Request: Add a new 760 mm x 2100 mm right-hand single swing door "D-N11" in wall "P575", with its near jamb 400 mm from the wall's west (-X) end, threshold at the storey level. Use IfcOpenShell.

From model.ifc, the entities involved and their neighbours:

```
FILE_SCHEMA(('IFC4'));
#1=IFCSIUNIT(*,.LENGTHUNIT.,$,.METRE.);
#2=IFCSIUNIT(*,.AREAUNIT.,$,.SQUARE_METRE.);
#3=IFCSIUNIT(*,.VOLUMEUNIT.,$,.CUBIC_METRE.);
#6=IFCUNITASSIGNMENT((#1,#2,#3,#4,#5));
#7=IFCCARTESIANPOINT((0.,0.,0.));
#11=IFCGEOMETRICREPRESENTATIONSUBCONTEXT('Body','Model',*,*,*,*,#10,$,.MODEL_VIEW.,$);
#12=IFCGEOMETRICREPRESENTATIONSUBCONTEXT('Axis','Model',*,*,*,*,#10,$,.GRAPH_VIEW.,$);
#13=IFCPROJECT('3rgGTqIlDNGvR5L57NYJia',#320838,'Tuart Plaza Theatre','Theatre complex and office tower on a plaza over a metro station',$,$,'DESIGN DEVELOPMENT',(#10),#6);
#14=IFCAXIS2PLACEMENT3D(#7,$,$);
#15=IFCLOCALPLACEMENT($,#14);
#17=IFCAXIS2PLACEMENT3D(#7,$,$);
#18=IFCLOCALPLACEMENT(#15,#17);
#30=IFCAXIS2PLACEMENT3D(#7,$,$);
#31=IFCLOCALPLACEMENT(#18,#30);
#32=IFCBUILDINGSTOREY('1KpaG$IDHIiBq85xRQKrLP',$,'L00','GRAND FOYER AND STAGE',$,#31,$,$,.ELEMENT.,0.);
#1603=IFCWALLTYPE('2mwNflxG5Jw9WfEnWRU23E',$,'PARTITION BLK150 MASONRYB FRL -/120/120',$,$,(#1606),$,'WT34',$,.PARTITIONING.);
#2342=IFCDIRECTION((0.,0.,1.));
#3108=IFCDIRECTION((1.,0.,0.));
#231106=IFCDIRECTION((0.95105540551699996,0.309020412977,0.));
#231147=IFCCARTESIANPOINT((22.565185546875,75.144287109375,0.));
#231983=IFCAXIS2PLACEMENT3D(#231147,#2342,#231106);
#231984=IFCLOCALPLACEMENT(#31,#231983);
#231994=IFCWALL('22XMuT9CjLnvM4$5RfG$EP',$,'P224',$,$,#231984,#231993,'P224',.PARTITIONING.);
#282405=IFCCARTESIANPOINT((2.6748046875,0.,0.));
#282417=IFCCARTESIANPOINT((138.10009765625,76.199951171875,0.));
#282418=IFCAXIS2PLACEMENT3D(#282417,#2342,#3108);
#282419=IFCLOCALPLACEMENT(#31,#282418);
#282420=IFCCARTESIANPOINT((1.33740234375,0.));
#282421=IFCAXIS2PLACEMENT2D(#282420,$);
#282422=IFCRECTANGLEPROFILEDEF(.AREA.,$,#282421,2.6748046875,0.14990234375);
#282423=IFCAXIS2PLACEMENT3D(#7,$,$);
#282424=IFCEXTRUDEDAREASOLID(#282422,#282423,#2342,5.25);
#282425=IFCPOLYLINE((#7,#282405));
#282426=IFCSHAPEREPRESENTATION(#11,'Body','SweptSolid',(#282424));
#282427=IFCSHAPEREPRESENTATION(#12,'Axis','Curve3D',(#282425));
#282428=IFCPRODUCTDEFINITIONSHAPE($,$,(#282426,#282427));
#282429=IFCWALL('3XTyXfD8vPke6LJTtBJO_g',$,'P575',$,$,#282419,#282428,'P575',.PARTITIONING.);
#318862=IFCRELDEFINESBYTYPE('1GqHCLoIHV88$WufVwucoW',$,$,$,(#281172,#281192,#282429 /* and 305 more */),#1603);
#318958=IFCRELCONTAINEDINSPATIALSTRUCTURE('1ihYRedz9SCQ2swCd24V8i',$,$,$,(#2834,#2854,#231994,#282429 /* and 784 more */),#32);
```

```python
import numpy as np
import ifcopenshell
import ifcopenshell.api.feature
import ifcopenshell.api.geometry
import ifcopenshell.api.root
import ifcopenshell.api.spatial
import ifcopenshell.geom
import ifcopenshell.util.element
import ifcopenshell.util.placement
import ifcopenshell.util.representation
import ifcopenshell.util.shape
import ifcopenshell.util.unit

model = ifcopenshell.open("model.ifc")
unit_scale = ifcopenshell.util.unit.calculate_unit_scale(model)
settings = ifcopenshell.geom.settings()


def volume(element):
    """Net volume in cubic metres, openings subtracted."""
    shape = ifcopenshell.geom.create_shape(settings, element)
    return ifcopenshell.util.shape.get_volume(shape.geometry)


wall = model.by_id(282429)
storey = ifcopenshell.util.element.get_container(wall, ifc_class="IfcBuildingStorey")
context = ifcopenshell.util.representation.get_context(model, "Model", "Body", "MODEL_VIEW")
before = volume(wall)

width, height, from_end, sill = 0.76, 2.1, 0.4, 0.0  # metres

# The wall runs along its own X axis, and the end named is its -X end.
wall_shape = ifcopenshell.geom.create_shape(settings, wall)
x, y, z = ifcopenshell.util.shape.get_vertices(wall_shape.geometry).T
start = x.min() + from_end
face, thickness = float(y.min()), float(y.max() - y.min())
wall_matrix = ifcopenshell.util.placement.get_local_placement(wall.ObjectPlacement)
level = ifcopenshell.util.placement.get_local_placement(storey.ObjectPlacement)[2, 3]


def in_wall(x, y):
    """Placement at x, y metres in the wall's axes, at sill height."""
    matrix = wall_matrix.copy()
    matrix[:, 3] = wall_matrix @ np.array([x / unit_scale, y / unit_scale, 0.0, 1.0])
    matrix[2, 3] = level + sill / unit_scale
    return matrix


# Opening: a box that overshoots both wall faces by 50 mm.
opening = ifcopenshell.api.root.create_entity(model, ifc_class="IfcOpeningElement", predefined_type="OPENING")
box = ifcopenshell.api.geometry.add_wall_representation(
    model, context=context, length=width, height=height, thickness=thickness + 0.1
)
ifcopenshell.api.geometry.assign_representation(model, product=opening, representation=box)
ifcopenshell.api.geometry.edit_object_placement(model, product=opening, matrix=in_wall(start, face - 0.05), is_si=False)
ifcopenshell.api.feature.add_feature(model, feature=opening, element=wall)

door = ifcopenshell.api.root.create_entity(model, ifc_class="IfcDoor", name="D-N11", predefined_type="DOOR")
door.OverallWidth, door.OverallHeight = width / unit_scale, height / unit_scale
door.OperationType = "SINGLE_SWING_RIGHT"
body = ifcopenshell.api.geometry.add_door_representation(
    model,
    context=context,
    overall_width=door.OverallWidth,
    overall_height=door.OverallHeight,
    operation_type="SINGLE_SWING_RIGHT",
    lining_properties={"LiningDepth": thickness / unit_scale, "ThresholdDepth": thickness / unit_scale},
)
ifcopenshell.api.geometry.assign_representation(model, product=door, representation=body)
ifcopenshell.api.spatial.assign_container(model, products=[door], relating_structure=storey)
ifcopenshell.api.feature.add_filling(model, opening=opening, element=door)

# The lining spans the wall, so the door starts at the wall face.
ifcopenshell.api.geometry.edit_object_placement(model, product=door, matrix=in_wall(start, face), is_si=False)

after = volume(wall)

print(f"wall volume {before:.3f} -> {after:.3f} m3")

model.write("model_updated.ifc")
```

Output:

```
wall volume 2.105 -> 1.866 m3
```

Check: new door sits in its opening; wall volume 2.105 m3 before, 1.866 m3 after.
